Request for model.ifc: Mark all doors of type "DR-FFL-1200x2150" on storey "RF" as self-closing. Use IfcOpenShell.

First a look at what the model holds.

```python
import ifcopenshell
import ifcopenshell.util.element

model = ifcopenshell.open("model.ifc")
print(model.schema)
storey = next(s for s in model.by_type("IfcBuildingStorey") if s.Name == "RF")
doors = [e for e in ifcopenshell.util.element.get_decomposition(storey) if e.is_a("IfcDoor")]
seen = {}
for e in doors:
    element_type = ifcopenshell.util.element.get_type(e)
    key = (element_type.Name if element_type != e and element_type else None, ifcopenshell.util.element.get_pset(e, "Pset_DoorCommon", "SelfClosing"))
    seen[key] = seen.get(key, 0) + 1
for (name, value), count in sorted(seen.items(), key=str):
    print(count, "x", name, "|", value)
```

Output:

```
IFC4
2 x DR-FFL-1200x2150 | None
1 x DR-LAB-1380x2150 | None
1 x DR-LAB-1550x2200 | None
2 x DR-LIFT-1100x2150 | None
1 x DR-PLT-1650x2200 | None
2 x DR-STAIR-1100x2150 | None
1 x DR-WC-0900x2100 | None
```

```python
import ifcopenshell
import ifcopenshell.api.pset
import ifcopenshell.util.element

model = ifcopenshell.open("model.ifc")

storey = next(s for s in model.by_type("IfcBuildingStorey") if s.Name == "RF")
doors = [e for e in ifcopenshell.util.element.get_decomposition(storey) if e.is_a("IfcDoor")]

count = 0
for e in doors:
    element_type = ifcopenshell.util.element.get_type(e)
    if element_type in (None, e) or element_type.Name != "DR-FFL-1200x2150":
        continue
    # add_pset returns the element's existing set when there is one.
    pset = ifcopenshell.api.pset.add_pset(model, product=e, name="Pset_DoorCommon")
    ifcopenshell.api.pset.edit_pset(model, pset=pset, properties={"SelfClosing": True})
    count += 1

print(count, "doors updated")

model.write("model_edited.ifc")
```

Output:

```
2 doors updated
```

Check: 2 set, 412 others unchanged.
